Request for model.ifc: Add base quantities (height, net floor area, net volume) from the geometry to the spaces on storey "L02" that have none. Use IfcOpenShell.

First a look at what the model holds.

```python
import ifcopenshell
import ifcopenshell.util.element
import ifcopenshell.util.unit

model = ifcopenshell.open("model.ifc")
print(model.schema)
for unit_type in ("LENGTHUNIT", "AREAUNIT", "VOLUMEUNIT"):
    print(unit_type, ifcopenshell.util.unit.calculate_unit_scale(model, unit_type))
storey = next(s for s in model.by_type("IfcBuildingStorey") if s.Name == "L02")
spaces = [e for e in ifcopenshell.util.element.get_decomposition(storey) if e.is_a("IfcSpace")]
for e in sorted(spaces, key=lambda e: e.id()):
    print(e.id(), e.is_a(), e.Name, list(ifcopenshell.util.element.get_psets(e, qtos_only=True)), sep=" | ")
```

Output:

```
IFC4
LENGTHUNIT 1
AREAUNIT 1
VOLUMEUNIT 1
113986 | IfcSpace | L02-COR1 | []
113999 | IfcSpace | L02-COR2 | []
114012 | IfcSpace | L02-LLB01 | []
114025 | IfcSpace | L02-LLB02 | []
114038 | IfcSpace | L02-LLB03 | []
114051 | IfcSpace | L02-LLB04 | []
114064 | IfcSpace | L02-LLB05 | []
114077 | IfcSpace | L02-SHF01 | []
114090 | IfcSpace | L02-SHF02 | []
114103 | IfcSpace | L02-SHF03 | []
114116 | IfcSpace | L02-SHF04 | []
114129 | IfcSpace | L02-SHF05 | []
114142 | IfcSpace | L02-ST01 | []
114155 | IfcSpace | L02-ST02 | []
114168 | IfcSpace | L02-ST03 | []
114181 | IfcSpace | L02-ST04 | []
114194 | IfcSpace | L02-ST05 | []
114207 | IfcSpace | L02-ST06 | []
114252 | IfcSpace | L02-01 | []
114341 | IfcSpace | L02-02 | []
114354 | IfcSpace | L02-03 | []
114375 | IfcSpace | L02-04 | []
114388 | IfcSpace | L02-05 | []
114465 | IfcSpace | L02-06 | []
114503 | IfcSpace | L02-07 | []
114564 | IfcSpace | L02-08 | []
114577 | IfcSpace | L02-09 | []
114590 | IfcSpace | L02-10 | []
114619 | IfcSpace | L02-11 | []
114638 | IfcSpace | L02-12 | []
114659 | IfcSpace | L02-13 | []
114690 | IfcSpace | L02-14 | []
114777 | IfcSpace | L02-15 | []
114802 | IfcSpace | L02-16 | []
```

```python
import ifcopenshell
import ifcopenshell.api.pset
import ifcopenshell.geom
import ifcopenshell.util.element
import ifcopenshell.util.shape
import ifcopenshell.util.unit

model = ifcopenshell.open("model.ifc")
unit_scale = ifcopenshell.util.unit.calculate_unit_scale(model)
area_scale = ifcopenshell.util.unit.calculate_unit_scale(model, "AREAUNIT")
volume_scale = ifcopenshell.util.unit.calculate_unit_scale(model, "VOLUMEUNIT")
settings = ifcopenshell.geom.settings()

storey = next(s for s in model.by_type("IfcBuildingStorey") if s.Name == "L02")
spaces = [e for e in ifcopenshell.util.element.get_decomposition(storey) if e.is_a("IfcSpace")]

for e in sorted(spaces, key=lambda e: e.id()):
    if ifcopenshell.util.element.get_psets(e, qtos_only=True, should_inherit=False):
        continue
    # Geometry comes back in metres, in the element's own axes.
    shape = ifcopenshell.geom.create_shape(settings, e)
    values = {
        "Height": ifcopenshell.util.shape.get_z(shape.geometry) / unit_scale,
        "NetFloorArea": ifcopenshell.util.shape.get_footprint_area(shape.geometry) / area_scale,
        "NetVolume": ifcopenshell.util.shape.get_volume(shape.geometry) / volume_scale,
    }
    qto = ifcopenshell.api.pset.add_qto(model, product=e, name="Qto_SpaceBaseQuantities")
    ifcopenshell.api.pset.edit_qto(model, qto=qto, properties=values)
    print(e.id(), {k: round(v, 3) for k, v in values.items()})

model.write("model_rev.ifc")
```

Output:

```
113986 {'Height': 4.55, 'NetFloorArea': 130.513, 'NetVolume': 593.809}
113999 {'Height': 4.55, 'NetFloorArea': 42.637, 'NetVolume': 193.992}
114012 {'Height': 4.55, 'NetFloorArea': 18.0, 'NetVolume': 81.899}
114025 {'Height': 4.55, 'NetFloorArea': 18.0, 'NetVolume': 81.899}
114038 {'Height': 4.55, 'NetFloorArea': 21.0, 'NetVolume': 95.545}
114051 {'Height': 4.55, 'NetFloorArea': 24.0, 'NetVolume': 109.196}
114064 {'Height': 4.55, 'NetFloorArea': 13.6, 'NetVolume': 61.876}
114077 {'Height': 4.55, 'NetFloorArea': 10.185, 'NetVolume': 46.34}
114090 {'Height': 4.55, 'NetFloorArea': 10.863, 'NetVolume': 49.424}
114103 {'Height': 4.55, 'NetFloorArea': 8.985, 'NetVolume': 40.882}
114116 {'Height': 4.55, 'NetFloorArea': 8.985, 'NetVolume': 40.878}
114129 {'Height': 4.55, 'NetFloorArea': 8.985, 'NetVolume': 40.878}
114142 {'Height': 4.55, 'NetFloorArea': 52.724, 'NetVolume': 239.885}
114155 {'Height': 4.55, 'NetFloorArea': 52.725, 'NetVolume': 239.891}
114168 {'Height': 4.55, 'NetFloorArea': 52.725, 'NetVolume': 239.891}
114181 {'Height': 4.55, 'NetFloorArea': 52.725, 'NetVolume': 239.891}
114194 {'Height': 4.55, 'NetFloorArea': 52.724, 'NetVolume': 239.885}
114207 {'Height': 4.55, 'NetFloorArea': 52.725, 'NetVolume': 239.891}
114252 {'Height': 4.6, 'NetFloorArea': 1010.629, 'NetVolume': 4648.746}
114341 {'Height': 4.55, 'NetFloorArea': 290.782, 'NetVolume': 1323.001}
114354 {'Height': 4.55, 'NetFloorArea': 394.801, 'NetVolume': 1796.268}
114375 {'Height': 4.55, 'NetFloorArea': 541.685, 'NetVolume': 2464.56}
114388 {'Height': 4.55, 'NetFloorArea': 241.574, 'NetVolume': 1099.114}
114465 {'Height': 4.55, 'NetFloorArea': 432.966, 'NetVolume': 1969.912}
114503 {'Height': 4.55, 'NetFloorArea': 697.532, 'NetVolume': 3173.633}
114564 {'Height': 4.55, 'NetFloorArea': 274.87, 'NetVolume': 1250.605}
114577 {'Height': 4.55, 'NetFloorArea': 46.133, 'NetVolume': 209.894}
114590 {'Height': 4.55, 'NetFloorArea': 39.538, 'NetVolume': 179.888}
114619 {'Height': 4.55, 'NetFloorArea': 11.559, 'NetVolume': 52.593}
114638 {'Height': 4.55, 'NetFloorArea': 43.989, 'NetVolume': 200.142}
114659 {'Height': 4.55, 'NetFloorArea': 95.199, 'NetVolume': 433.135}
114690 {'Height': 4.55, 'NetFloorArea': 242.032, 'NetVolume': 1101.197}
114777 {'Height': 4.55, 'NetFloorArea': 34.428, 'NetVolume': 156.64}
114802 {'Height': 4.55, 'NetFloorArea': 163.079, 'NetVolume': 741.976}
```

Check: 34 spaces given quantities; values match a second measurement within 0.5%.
